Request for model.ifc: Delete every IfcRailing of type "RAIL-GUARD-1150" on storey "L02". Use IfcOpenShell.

First a look at what the model holds.

```python
import ifcopenshell
import ifcopenshell.util.element

model = ifcopenshell.open("model.ifc")
print(model.schema)
storey = next(s for s in model.by_type("IfcBuildingStorey") if s.Name == "L02")
railings = [e for e in ifcopenshell.util.element.get_decomposition(storey) if e.is_a("IfcRailing")]
seen = {}
for e in railings:
    element_type = ifcopenshell.util.element.get_type(e)
    name = element_type.Name if element_type not in (None, e) else None
    seen[name] = seen.get(name, 0) + 1
for name, count in sorted(seen.items(), key=str):
    print(count, "x", name)
```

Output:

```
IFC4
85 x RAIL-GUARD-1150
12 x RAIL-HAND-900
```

```python
import ifcopenshell
import ifcopenshell.api.root
import ifcopenshell.util.element

model = ifcopenshell.open("model.ifc")

storey = next(s for s in model.by_type("IfcBuildingStorey") if s.Name == "L02")
railings = [e for e in ifcopenshell.util.element.get_decomposition(storey) if e.is_a("IfcRailing")]
targets = [e for e in railings if (t := ifcopenshell.util.element.get_type(e)) not in (None, e) and t.Name == "RAIL-GUARD-1150"]

for e in targets:
    ifcopenshell.api.root.remove_product(model, product=e)
print(len(targets), "removed")

model.write("model-out.ifc")
```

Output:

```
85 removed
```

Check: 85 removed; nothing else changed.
